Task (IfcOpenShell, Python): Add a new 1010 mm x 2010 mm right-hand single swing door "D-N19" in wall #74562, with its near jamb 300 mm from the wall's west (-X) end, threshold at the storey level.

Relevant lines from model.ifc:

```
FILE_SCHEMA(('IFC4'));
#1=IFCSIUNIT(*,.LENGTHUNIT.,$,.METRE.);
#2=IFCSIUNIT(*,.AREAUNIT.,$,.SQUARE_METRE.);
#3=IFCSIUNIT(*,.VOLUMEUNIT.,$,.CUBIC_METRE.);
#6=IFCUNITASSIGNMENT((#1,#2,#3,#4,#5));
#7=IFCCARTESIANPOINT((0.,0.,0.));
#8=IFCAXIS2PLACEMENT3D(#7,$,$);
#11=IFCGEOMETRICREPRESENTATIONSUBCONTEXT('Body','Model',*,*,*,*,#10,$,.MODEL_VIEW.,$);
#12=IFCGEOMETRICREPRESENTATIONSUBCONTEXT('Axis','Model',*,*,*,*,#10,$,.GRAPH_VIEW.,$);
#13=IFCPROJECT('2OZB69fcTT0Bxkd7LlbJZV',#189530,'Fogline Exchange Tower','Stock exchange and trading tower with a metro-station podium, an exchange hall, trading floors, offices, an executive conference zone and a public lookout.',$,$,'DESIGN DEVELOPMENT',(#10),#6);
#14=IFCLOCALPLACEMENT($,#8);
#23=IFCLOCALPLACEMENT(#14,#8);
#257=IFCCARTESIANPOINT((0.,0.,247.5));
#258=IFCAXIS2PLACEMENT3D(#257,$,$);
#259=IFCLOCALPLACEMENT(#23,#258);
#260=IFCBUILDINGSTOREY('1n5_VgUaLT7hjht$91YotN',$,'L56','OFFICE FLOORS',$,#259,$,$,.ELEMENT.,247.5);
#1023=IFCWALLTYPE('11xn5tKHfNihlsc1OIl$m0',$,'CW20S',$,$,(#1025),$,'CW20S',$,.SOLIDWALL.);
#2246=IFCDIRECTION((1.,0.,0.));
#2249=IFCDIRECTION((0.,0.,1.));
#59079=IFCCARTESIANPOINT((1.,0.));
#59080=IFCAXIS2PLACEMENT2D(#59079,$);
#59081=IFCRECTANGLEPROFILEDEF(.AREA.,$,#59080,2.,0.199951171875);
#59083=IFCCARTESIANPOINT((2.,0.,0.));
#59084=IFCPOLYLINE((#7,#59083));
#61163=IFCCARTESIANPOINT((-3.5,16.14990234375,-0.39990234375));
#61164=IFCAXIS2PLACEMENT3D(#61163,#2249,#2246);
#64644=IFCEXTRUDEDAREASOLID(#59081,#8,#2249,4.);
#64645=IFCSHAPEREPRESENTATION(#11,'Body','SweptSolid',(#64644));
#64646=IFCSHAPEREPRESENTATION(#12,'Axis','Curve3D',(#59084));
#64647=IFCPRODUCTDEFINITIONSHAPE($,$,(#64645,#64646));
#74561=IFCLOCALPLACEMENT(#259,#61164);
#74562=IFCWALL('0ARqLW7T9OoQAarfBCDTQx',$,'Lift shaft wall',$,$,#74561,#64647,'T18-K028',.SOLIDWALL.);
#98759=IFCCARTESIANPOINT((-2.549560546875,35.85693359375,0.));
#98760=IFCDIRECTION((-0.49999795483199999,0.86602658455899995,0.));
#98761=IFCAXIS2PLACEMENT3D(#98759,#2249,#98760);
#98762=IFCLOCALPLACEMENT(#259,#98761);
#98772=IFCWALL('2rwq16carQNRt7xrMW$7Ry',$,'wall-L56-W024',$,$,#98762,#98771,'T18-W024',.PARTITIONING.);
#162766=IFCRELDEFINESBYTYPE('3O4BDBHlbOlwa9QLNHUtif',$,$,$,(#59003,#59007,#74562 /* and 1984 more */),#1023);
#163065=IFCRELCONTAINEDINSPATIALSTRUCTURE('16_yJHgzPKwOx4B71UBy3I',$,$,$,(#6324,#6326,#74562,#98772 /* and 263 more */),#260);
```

```python
import numpy as np
import ifcopenshell
import ifcopenshell.api.feature
import ifcopenshell.api.geometry
import ifcopenshell.api.root
import ifcopenshell.api.spatial
import ifcopenshell.geom
import ifcopenshell.util.element
import ifcopenshell.util.placement
import ifcopenshell.util.representation
import ifcopenshell.util.shape
import ifcopenshell.util.unit

model = ifcopenshell.open("model.ifc")
unit_scale = ifcopenshell.util.unit.calculate_unit_scale(model)
settings = ifcopenshell.geom.settings()


def volume(element):
    """Net volume in cubic metres, openings subtracted."""
    shape = ifcopenshell.geom.create_shape(settings, element)
    return ifcopenshell.util.shape.get_volume(shape.geometry)


wall = model.by_id(74562)
storey = ifcopenshell.util.element.get_container(wall, ifc_class="IfcBuildingStorey")
context = ifcopenshell.util.representation.get_context(model, "Model", "Body", "MODEL_VIEW")
before = volume(wall)

width, height, from_end, sill = 1.01, 2.01, 0.3, 0.0  # metres

# The wall runs along its own X axis, and the end named is its -X end.
wall_shape = ifcopenshell.geom.create_shape(settings, wall)
x, y, z = ifcopenshell.util.shape.get_vertices(wall_shape.geometry).T
start = x.min() + from_end
face, thickness = float(y.min()), float(y.max() - y.min())
wall_matrix = ifcopenshell.util.placement.get_local_placement(wall.ObjectPlacement)
level = ifcopenshell.util.placement.get_local_placement(storey.ObjectPlacement)[2, 3]


def in_wall(x, y):
    """Placement at x, y metres in the wall's axes, at sill height."""
    matrix = wall_matrix.copy()
    matrix[:, 3] = wall_matrix @ np.array([x / unit_scale, y / unit_scale, 0.0, 1.0])
    matrix[2, 3] = level + sill / unit_scale
    return matrix


# Opening: a box that overshoots both wall faces by 50 mm.
opening = ifcopenshell.api.root.create_entity(model, ifc_class="IfcOpeningElement", predefined_type="OPENING")
box = ifcopenshell.api.geometry.add_wall_representation(
    model, context=context, length=width, height=height, thickness=thickness + 0.1
)
ifcopenshell.api.geometry.assign_representation(model, product=opening, representation=box)
ifcopenshell.api.geometry.edit_object_placement(model, product=opening, matrix=in_wall(start, face - 0.05), is_si=False)
ifcopenshell.api.feature.add_feature(model, feature=opening, element=wall)

door = ifcopenshell.api.root.create_entity(model, ifc_class="IfcDoor", name="D-N19", predefined_type="DOOR")
door.OverallWidth, door.OverallHeight = width / unit_scale, height / unit_scale
door.OperationType = "SINGLE_SWING_RIGHT"
body = ifcopenshell.api.geometry.add_door_representation(
    model,
    context=context,
    overall_width=door.OverallWidth,
    overall_height=door.OverallHeight,
    operation_type="SINGLE_SWING_RIGHT",
    lining_properties={"LiningDepth": thickness / unit_scale, "ThresholdDepth": thickness / unit_scale},
)
ifcopenshell.api.geometry.assign_representation(model, product=door, representation=body)
ifcopenshell.api.spatial.assign_container(model, products=[door], relating_structure=storey)
ifcopenshell.api.feature.add_filling(model, opening=opening, element=door)

# The lining spans the wall, so the door starts at the wall face.
ifcopenshell.api.geometry.edit_object_placement(model, product=door, matrix=in_wall(start, face), is_si=False)

after = volume(wall)

print(f"wall volume {before:.3f} -> {after:.3f} m3")

model.write("model-out.ifc")
```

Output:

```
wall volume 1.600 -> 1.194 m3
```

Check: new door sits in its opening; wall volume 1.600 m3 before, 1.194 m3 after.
